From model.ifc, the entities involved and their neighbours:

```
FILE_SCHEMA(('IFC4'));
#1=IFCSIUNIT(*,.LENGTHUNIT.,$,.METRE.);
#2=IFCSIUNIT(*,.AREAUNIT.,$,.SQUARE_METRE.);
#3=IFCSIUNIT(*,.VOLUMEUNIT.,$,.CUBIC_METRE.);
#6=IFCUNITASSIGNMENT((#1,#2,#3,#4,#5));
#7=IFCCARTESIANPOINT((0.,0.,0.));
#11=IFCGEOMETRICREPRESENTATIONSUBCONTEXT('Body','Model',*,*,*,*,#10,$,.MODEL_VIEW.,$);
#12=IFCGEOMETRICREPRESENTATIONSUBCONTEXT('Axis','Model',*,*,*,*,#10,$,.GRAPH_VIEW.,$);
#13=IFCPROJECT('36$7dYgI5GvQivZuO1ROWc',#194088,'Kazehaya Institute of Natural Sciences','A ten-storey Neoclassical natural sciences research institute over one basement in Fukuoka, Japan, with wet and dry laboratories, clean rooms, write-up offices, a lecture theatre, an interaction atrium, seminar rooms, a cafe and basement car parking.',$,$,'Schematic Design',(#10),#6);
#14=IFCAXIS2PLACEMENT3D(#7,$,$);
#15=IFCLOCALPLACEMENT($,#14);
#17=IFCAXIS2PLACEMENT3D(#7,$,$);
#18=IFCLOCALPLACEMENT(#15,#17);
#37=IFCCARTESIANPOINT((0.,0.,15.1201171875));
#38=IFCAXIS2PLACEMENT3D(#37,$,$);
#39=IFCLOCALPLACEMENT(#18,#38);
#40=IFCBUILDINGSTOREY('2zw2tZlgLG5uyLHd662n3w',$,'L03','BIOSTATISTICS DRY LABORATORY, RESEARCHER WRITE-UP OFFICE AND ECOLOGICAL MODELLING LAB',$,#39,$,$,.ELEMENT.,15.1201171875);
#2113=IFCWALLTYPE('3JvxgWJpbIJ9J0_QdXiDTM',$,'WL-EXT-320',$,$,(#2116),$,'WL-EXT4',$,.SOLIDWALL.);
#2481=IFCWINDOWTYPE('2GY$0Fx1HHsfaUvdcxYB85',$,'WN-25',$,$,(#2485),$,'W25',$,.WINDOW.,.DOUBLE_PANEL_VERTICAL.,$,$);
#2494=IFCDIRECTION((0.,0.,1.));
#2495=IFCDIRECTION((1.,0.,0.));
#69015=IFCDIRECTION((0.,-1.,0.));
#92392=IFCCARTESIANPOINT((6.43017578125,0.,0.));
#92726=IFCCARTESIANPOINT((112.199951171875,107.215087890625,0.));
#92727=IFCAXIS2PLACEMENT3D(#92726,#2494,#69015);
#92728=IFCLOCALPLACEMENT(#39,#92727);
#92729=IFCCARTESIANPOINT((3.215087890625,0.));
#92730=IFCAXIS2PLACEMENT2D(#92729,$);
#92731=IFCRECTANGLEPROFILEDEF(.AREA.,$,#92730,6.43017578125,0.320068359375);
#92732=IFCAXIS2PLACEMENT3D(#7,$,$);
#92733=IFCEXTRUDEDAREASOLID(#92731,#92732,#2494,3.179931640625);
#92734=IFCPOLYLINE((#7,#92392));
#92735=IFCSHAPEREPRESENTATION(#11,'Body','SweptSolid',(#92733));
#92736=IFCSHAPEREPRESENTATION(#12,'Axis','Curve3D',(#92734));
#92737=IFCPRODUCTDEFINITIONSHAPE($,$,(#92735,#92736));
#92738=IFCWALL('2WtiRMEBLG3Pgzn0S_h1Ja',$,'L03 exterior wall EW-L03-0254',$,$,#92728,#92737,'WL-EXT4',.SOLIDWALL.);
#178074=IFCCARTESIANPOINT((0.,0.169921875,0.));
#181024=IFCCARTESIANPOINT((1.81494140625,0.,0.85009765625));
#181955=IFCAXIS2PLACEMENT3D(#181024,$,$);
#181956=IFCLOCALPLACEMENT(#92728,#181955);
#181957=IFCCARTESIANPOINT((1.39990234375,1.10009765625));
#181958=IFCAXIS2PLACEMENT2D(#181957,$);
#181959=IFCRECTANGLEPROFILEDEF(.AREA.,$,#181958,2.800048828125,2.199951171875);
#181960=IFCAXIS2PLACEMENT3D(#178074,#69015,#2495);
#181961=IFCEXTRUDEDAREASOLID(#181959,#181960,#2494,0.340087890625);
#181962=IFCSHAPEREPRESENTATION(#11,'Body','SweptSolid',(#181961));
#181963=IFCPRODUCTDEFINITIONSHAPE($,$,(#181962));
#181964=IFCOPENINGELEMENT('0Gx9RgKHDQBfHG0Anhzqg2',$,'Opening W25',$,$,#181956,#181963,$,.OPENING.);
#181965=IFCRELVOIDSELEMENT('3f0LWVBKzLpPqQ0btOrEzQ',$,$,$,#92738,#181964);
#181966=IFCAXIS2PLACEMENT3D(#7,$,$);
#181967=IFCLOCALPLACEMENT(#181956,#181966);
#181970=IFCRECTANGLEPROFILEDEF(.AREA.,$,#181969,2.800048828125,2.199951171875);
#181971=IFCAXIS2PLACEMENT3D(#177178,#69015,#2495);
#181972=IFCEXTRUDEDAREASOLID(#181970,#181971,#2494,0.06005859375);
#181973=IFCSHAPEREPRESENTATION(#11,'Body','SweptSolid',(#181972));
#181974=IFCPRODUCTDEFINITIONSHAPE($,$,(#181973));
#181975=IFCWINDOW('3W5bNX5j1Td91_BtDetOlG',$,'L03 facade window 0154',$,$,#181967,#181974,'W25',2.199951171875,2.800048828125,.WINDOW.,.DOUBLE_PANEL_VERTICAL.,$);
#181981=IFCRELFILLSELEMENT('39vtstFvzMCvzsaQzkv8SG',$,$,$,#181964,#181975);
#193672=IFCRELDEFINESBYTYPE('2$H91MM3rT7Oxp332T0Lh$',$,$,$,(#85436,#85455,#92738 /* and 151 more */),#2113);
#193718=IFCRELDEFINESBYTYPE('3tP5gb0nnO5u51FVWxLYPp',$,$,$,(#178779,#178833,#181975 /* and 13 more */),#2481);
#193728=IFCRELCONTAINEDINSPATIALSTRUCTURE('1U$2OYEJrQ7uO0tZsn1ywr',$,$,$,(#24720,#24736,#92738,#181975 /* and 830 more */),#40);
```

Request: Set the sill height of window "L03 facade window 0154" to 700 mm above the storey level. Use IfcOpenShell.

```python
import numpy as np
import ifcopenshell
import ifcopenshell.api.geometry
import ifcopenshell.geom
import ifcopenshell.util.element
import ifcopenshell.util.placement
import ifcopenshell.util.shape
import ifcopenshell.util.unit

model = ifcopenshell.open("model.ifc")
unit_scale = ifcopenshell.util.unit.calculate_unit_scale(model)

window = model.by_id(181975)
opening = window.FillsVoids[0].RelatingOpeningElement
storey = ifcopenshell.util.element.get_container(window, ifc_class="IfcBuildingStorey")
level = ifcopenshell.util.placement.get_local_placement(storey.ObjectPlacement)[2, 3]

# The opening's origin need not be at the sill, so measure its lowest point.
shape = ifcopenshell.geom.create_shape(ifcopenshell.geom.settings(), opening)
bottom = ifcopenshell.util.shape.get_shape_bottom_elevation(shape, shape.geometry) / unit_scale
dz = level + 0.7 / unit_scale - bottom

shift = np.array([0.0, 0.0, dz])
# The window is placed relative to its opening, so it follows when the opening moves.
matrix = ifcopenshell.util.placement.get_local_placement(opening.ObjectPlacement)
matrix[:3, 3] += shift
ifcopenshell.api.geometry.edit_object_placement(
    model, product=opening, matrix=matrix, is_si=False, should_transform_children=True
)

print(f"moved by {dz * unit_scale:+.3f} m")

model.write("model_rev.ifc")
```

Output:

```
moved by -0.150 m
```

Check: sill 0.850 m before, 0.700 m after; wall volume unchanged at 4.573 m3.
